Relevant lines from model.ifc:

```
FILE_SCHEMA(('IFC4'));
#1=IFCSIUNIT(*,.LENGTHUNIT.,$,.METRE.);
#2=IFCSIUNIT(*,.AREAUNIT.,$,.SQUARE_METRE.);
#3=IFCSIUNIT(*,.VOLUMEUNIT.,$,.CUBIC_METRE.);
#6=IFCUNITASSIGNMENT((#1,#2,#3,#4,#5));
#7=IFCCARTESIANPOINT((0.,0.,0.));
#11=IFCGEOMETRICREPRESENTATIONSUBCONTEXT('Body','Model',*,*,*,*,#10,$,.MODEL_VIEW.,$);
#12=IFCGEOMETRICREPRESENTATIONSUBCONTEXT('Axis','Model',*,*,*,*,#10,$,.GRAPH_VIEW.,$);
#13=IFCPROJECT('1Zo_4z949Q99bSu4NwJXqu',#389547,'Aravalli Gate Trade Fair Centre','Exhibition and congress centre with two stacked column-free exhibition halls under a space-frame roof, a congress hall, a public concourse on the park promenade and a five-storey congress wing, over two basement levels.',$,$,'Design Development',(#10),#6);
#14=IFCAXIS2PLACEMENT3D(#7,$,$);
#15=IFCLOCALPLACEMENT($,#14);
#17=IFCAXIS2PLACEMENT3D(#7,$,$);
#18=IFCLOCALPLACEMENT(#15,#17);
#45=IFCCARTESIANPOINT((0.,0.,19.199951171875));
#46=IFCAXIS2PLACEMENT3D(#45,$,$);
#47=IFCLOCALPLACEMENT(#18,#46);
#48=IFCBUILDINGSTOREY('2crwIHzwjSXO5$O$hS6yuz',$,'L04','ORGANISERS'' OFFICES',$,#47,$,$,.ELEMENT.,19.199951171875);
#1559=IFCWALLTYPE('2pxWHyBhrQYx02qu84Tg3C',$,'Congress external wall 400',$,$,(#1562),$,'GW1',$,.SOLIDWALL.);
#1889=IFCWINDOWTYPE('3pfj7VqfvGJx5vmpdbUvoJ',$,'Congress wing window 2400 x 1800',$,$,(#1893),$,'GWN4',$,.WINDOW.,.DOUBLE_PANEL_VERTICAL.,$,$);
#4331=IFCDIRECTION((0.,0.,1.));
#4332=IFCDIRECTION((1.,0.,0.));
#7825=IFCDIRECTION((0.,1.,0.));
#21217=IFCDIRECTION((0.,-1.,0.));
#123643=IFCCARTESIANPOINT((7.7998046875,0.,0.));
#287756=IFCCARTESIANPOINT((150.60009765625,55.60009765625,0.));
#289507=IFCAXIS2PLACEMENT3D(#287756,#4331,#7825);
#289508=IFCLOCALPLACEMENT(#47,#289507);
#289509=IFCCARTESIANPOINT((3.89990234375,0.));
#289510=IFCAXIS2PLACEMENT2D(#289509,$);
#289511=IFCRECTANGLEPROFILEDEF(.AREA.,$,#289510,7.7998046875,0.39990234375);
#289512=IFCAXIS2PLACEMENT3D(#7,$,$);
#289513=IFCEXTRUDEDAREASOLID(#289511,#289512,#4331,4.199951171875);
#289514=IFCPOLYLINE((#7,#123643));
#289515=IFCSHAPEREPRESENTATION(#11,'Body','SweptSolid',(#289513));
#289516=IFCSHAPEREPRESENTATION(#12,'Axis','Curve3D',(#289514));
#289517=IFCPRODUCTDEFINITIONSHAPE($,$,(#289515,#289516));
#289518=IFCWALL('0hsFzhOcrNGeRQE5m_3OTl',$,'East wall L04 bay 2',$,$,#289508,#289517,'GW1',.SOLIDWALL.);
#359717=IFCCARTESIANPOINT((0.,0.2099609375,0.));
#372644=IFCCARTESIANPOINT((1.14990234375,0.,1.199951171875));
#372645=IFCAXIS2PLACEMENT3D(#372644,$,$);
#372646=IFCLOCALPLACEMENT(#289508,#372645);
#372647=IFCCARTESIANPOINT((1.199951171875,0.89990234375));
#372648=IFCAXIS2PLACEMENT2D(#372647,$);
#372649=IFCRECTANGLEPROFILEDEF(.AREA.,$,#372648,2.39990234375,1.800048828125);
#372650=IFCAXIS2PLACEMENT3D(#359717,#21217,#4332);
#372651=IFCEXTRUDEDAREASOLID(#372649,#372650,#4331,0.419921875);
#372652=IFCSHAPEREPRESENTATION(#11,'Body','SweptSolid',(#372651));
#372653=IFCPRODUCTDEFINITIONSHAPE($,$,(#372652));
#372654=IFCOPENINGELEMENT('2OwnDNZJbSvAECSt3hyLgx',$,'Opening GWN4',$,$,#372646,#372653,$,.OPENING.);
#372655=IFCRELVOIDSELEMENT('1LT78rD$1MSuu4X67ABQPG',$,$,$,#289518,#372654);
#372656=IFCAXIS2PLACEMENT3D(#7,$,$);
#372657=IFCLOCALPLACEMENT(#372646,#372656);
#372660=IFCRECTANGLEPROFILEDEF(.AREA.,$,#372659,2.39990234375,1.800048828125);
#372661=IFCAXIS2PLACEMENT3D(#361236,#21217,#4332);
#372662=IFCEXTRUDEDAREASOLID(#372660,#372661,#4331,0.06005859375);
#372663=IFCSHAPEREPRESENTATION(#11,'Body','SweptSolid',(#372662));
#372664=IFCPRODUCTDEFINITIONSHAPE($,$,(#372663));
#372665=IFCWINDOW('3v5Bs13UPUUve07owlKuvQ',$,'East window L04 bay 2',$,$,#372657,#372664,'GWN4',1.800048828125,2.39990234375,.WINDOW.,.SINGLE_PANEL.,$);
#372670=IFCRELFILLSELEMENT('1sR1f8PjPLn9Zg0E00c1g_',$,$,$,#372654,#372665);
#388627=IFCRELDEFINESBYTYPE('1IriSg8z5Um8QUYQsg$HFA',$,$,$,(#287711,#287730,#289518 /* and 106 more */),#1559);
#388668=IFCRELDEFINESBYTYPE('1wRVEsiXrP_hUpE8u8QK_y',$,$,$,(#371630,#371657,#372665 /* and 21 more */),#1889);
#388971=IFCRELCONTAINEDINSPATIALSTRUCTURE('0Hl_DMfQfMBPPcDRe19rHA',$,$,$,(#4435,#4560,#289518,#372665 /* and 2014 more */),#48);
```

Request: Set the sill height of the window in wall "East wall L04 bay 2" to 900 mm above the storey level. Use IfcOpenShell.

```python
import numpy as np
import ifcopenshell
import ifcopenshell.api.geometry
import ifcopenshell.geom
import ifcopenshell.util.element
import ifcopenshell.util.placement
import ifcopenshell.util.shape
import ifcopenshell.util.unit

model = ifcopenshell.open("model.ifc")
unit_scale = ifcopenshell.util.unit.calculate_unit_scale(model)

window = model.by_id(372665)
opening = window.FillsVoids[0].RelatingOpeningElement
storey = ifcopenshell.util.element.get_container(window, ifc_class="IfcBuildingStorey")
level = ifcopenshell.util.placement.get_local_placement(storey.ObjectPlacement)[2, 3]

# The opening's origin need not be at the sill, so measure its lowest point.
shape = ifcopenshell.geom.create_shape(ifcopenshell.geom.settings(), opening)
bottom = ifcopenshell.util.shape.get_shape_bottom_elevation(shape, shape.geometry) / unit_scale
dz = level + 0.9 / unit_scale - bottom

shift = np.array([0.0, 0.0, dz])
# The window is placed relative to its opening, so it follows when the opening moves.
matrix = ifcopenshell.util.placement.get_local_placement(opening.ObjectPlacement)
matrix[:3, 3] += shift
ifcopenshell.api.geometry.edit_object_placement(
    model, product=opening, matrix=matrix, is_si=False, should_transform_children=True
)

print(f"moved by {dz * unit_scale:+.3f} m")

model.write("model-out.ifc")
```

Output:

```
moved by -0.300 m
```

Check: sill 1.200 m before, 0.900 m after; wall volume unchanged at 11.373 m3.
